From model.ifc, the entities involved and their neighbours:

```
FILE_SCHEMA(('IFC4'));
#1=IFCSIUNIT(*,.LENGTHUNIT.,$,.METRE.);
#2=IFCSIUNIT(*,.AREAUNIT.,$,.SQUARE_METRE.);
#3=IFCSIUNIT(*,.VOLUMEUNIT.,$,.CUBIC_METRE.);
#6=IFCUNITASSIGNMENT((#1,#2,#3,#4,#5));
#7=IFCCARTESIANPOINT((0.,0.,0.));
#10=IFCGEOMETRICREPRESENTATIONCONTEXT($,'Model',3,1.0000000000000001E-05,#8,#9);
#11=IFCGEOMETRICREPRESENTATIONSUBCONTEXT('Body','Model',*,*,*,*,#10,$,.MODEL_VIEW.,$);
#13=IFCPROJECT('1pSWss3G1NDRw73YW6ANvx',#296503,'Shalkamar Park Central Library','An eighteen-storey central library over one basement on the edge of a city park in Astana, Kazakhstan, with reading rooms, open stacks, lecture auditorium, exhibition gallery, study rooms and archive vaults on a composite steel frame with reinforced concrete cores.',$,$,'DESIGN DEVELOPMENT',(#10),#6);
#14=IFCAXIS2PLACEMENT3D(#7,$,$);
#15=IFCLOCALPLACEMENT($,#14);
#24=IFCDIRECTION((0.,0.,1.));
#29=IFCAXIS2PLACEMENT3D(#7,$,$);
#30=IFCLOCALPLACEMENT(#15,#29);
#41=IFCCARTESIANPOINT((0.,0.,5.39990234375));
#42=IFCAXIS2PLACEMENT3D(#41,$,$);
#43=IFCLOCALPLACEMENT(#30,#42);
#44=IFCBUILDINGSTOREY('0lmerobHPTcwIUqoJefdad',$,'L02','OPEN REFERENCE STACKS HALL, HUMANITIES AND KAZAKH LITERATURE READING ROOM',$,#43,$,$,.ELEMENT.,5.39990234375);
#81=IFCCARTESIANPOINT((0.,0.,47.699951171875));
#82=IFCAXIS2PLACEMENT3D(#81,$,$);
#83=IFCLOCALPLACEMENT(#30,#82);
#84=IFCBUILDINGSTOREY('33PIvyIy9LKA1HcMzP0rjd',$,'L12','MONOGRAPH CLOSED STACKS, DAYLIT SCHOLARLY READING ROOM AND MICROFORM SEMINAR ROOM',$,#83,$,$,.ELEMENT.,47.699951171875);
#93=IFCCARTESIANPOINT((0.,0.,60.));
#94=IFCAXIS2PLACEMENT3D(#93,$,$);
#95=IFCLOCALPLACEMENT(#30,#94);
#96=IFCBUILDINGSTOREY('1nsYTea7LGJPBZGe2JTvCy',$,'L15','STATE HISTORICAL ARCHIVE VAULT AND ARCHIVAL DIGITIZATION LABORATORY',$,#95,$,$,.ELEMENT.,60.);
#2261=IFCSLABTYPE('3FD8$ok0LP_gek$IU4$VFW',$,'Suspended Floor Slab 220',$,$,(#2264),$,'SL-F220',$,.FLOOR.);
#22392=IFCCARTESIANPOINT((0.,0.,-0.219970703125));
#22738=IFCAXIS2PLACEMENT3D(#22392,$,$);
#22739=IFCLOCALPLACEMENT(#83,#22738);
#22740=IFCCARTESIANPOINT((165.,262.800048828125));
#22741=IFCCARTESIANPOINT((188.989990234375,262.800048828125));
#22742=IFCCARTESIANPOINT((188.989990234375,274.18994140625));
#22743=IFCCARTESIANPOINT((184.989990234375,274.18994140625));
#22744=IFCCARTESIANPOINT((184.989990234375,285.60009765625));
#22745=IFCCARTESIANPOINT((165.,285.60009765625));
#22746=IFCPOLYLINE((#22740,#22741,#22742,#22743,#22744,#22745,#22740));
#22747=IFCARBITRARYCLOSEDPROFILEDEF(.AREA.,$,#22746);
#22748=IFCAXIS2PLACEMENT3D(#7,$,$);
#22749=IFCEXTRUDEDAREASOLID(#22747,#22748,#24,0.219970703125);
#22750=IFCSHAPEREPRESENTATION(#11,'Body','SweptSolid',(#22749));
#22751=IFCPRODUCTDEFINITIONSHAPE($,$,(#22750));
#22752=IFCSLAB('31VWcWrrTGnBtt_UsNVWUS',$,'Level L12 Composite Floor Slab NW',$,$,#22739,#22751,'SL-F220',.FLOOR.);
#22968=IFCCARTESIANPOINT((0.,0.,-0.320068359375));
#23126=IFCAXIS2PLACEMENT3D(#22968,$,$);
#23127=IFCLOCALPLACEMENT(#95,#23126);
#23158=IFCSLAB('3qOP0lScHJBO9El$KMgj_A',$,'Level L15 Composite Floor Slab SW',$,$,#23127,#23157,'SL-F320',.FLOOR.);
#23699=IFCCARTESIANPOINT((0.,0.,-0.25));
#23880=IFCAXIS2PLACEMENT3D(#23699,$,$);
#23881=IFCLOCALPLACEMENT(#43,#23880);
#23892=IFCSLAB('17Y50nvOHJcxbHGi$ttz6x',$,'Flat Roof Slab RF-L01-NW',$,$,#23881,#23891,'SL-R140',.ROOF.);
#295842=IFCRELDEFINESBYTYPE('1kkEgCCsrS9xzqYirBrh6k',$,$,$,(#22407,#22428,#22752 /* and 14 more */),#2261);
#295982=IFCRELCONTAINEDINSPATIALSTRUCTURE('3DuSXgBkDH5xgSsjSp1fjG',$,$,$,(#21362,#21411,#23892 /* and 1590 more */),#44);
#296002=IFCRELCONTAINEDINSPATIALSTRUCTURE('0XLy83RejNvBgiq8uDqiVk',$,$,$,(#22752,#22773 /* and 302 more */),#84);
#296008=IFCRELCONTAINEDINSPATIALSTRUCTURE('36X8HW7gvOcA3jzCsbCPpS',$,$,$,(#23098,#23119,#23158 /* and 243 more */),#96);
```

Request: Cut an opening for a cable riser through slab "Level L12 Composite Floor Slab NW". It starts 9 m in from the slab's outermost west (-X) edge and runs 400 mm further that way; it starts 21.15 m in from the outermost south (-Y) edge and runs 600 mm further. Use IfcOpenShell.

```python
import numpy as np
import ifcopenshell
import ifcopenshell.api.feature
import ifcopenshell.api.geometry
import ifcopenshell.api.root
import ifcopenshell.geom
import ifcopenshell.util.placement
import ifcopenshell.util.representation
import ifcopenshell.util.shape
import ifcopenshell.util.unit

model = ifcopenshell.open("model.ifc")
unit_scale = ifcopenshell.util.unit.calculate_unit_scale(model)
settings = ifcopenshell.geom.settings()


def volume(element):
    """Net volume in cubic metres, openings subtracted."""
    shape = ifcopenshell.geom.create_shape(settings, element)
    return ifcopenshell.util.shape.get_volume(shape.geometry)


slab = model.by_id(22752)
before = volume(slab)

# Extent in the slab's own axes, in metres. The edges named are its -X and -Y sides.
slab_shape = ifcopenshell.geom.create_shape(settings, slab)
vertices = ifcopenshell.util.shape.get_vertices(slab_shape.geometry)
x_min, y_min, bottom = vertices.min(axis=0)
top = vertices[:, 2].max()

opening = ifcopenshell.api.root.create_entity(model, ifc_class="IfcOpeningElement", name="Cable riser opening", predefined_type="OPENING")
context = ifcopenshell.util.representation.get_context(model, "Model", "Body", "MODEL_VIEW")
width, depth = 0.4, 0.6
outline = [(0.0, 0.0), (width, 0.0), (width, depth), (0.0, depth), (0.0, 0.0)]
# Overshoot both faces by 50 mm so the cut is clean.
shape = ifcopenshell.api.geometry.add_slab_representation(
    model, context=context, depth=top - bottom + 0.1, polyline=outline
)
ifcopenshell.api.geometry.assign_representation(model, product=opening, representation=shape)

matrix = ifcopenshell.util.placement.get_local_placement(slab.ObjectPlacement)
matrix[:, 3] = matrix @ np.append(np.array([x_min + 9, y_min + 21.15, bottom - 0.05]) / unit_scale, 1.0)
ifcopenshell.api.geometry.edit_object_placement(model, product=opening, matrix=matrix, is_si=False)
ifcopenshell.api.feature.add_feature(model, feature=opening, element=slab)

after = volume(slab)

print(f"slab volume {before:.3f} -> {after:.3f} m3")

model.write("model_updated.ifc")
```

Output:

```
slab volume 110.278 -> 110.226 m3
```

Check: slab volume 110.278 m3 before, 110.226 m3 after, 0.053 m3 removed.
